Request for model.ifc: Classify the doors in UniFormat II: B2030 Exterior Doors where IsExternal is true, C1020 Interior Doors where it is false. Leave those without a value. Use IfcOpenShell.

First a look at what the model holds.

```python
import ifcopenshell
import ifcopenshell.util.element

model = ifcopenshell.open("model.ifc")
print(model.schema)
print("classifications:", [c.Name for c in model.by_type("IfcClassification")])
values = [ifcopenshell.util.element.get_pset(e, "Pset_DoorCommon", "IsExternal") for e in model.by_type("IfcDoor")]
for value in (True, False, None):
    print("IsExternal", value, values.count(value))
```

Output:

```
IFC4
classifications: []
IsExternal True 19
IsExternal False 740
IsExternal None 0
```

```python
import ifcopenshell
import ifcopenshell.api.classification
import ifcopenshell.util.element

model = ifcopenshell.open("model.ifc")

system = ifcopenshell.api.classification.add_classification(model, classification="UniFormat II")

doors = model.by_type("IfcDoor")
external = {e: ifcopenshell.util.element.get_pset(e, "Pset_DoorCommon", "IsExternal") for e in doors}
for flag, code, name in ((True, "B2030", "Exterior Doors"), (False, "C1020", "Interior Doors")):
    products = [e for e in doors if external[e] is flag]
    ifcopenshell.api.classification.add_reference(
        model, products=products, classification=system, identification=code, name=name
    )
    print(code, len(products))

model.write("model_updated.ifc")
```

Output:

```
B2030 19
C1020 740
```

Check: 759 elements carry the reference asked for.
